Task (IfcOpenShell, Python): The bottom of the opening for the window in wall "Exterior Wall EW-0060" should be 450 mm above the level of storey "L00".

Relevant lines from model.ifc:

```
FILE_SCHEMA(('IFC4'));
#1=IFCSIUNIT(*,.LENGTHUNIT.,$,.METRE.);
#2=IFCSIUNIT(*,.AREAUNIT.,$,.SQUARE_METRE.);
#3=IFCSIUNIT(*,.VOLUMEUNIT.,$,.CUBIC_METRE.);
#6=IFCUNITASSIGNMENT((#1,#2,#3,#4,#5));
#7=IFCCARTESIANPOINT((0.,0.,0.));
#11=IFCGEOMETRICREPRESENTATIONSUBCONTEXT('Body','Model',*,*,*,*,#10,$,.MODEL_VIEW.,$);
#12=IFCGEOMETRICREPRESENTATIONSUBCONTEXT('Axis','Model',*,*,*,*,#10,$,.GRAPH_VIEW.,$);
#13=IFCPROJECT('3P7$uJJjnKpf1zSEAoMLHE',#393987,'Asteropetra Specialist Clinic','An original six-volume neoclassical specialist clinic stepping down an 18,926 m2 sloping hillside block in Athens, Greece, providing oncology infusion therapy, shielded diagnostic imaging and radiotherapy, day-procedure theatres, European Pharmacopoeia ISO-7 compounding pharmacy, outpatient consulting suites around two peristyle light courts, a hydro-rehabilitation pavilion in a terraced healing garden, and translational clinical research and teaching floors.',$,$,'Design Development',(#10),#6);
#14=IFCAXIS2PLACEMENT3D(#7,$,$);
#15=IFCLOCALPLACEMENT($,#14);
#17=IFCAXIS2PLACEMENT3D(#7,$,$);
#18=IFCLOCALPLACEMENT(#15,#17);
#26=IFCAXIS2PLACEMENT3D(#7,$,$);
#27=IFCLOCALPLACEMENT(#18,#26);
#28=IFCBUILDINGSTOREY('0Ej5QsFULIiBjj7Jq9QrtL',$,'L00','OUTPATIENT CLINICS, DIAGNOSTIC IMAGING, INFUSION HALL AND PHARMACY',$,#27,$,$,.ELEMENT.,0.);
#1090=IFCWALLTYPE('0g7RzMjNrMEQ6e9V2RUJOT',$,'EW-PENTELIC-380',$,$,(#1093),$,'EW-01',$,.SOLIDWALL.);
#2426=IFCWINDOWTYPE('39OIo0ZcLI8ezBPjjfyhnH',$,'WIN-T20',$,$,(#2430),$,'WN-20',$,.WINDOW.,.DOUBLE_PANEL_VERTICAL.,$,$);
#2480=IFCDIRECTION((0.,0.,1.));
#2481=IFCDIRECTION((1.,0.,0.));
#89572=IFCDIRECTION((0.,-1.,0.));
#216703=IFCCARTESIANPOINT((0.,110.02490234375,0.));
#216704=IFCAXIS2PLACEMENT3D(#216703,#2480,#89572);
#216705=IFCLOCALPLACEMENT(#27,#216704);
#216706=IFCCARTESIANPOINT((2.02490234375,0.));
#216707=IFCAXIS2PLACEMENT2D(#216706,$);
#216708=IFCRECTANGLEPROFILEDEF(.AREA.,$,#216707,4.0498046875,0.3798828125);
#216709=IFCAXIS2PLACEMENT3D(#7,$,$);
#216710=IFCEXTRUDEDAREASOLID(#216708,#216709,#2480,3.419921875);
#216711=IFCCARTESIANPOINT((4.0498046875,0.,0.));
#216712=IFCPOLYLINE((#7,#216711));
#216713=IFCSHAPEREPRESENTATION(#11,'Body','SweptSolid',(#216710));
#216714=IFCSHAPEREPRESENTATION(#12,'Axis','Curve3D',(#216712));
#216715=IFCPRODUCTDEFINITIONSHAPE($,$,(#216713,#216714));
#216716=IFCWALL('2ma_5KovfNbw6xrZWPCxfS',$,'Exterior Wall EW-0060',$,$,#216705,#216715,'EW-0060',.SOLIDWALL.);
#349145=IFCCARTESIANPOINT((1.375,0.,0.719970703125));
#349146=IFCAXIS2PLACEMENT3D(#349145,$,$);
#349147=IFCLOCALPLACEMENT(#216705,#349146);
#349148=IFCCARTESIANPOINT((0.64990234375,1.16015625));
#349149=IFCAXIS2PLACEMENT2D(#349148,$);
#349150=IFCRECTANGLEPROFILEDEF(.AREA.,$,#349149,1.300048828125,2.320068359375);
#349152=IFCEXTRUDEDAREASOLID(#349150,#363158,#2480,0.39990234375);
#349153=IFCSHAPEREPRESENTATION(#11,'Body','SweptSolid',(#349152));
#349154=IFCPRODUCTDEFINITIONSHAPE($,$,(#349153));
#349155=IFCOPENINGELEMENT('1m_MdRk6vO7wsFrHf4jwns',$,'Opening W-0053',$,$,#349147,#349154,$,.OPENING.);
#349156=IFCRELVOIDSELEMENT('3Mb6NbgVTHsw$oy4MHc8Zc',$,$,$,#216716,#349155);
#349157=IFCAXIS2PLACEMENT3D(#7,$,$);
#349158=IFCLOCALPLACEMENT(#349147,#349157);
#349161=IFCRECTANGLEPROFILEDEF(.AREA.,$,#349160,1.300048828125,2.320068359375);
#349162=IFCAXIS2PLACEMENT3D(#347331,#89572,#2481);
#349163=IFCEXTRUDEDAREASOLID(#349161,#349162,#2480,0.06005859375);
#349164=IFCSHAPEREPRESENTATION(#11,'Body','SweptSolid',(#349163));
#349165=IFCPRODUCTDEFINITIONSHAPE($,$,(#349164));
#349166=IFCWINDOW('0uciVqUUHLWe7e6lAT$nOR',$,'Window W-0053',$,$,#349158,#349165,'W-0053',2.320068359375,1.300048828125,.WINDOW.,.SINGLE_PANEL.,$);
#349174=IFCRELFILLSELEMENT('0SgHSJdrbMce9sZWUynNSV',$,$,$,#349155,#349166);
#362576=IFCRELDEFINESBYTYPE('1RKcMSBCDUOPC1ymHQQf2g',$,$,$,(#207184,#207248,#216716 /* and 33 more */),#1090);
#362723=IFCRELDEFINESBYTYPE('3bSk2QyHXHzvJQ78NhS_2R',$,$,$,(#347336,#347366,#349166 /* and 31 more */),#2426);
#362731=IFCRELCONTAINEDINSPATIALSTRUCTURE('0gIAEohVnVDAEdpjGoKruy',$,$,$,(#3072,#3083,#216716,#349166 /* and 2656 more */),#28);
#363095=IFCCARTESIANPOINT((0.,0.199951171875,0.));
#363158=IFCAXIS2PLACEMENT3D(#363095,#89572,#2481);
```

```python
import numpy as np
import ifcopenshell
import ifcopenshell.api.geometry
import ifcopenshell.geom
import ifcopenshell.util.element
import ifcopenshell.util.placement
import ifcopenshell.util.shape
import ifcopenshell.util.unit

model = ifcopenshell.open("model.ifc")
unit_scale = ifcopenshell.util.unit.calculate_unit_scale(model)

window = model.by_id(349166)
opening = window.FillsVoids[0].RelatingOpeningElement
storey = ifcopenshell.util.element.get_container(window, ifc_class="IfcBuildingStorey")
level = ifcopenshell.util.placement.get_local_placement(storey.ObjectPlacement)[2, 3]

# The opening's origin need not be at the sill, so measure its lowest point.
shape = ifcopenshell.geom.create_shape(ifcopenshell.geom.settings(), opening)
bottom = ifcopenshell.util.shape.get_shape_bottom_elevation(shape, shape.geometry) / unit_scale
dz = level + 0.45 / unit_scale - bottom

shift = np.array([0.0, 0.0, dz])
# The window is placed relative to its opening, so it follows when the opening moves.
matrix = ifcopenshell.util.placement.get_local_placement(opening.ObjectPlacement)
matrix[:3, 3] += shift
ifcopenshell.api.geometry.edit_object_placement(
    model, product=opening, matrix=matrix, is_si=False, should_transform_children=True
)

print(f"moved by {dz * unit_scale:+.3f} m")

model.write("model_v2.ifc")
```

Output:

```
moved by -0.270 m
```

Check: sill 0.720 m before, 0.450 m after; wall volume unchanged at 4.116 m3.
